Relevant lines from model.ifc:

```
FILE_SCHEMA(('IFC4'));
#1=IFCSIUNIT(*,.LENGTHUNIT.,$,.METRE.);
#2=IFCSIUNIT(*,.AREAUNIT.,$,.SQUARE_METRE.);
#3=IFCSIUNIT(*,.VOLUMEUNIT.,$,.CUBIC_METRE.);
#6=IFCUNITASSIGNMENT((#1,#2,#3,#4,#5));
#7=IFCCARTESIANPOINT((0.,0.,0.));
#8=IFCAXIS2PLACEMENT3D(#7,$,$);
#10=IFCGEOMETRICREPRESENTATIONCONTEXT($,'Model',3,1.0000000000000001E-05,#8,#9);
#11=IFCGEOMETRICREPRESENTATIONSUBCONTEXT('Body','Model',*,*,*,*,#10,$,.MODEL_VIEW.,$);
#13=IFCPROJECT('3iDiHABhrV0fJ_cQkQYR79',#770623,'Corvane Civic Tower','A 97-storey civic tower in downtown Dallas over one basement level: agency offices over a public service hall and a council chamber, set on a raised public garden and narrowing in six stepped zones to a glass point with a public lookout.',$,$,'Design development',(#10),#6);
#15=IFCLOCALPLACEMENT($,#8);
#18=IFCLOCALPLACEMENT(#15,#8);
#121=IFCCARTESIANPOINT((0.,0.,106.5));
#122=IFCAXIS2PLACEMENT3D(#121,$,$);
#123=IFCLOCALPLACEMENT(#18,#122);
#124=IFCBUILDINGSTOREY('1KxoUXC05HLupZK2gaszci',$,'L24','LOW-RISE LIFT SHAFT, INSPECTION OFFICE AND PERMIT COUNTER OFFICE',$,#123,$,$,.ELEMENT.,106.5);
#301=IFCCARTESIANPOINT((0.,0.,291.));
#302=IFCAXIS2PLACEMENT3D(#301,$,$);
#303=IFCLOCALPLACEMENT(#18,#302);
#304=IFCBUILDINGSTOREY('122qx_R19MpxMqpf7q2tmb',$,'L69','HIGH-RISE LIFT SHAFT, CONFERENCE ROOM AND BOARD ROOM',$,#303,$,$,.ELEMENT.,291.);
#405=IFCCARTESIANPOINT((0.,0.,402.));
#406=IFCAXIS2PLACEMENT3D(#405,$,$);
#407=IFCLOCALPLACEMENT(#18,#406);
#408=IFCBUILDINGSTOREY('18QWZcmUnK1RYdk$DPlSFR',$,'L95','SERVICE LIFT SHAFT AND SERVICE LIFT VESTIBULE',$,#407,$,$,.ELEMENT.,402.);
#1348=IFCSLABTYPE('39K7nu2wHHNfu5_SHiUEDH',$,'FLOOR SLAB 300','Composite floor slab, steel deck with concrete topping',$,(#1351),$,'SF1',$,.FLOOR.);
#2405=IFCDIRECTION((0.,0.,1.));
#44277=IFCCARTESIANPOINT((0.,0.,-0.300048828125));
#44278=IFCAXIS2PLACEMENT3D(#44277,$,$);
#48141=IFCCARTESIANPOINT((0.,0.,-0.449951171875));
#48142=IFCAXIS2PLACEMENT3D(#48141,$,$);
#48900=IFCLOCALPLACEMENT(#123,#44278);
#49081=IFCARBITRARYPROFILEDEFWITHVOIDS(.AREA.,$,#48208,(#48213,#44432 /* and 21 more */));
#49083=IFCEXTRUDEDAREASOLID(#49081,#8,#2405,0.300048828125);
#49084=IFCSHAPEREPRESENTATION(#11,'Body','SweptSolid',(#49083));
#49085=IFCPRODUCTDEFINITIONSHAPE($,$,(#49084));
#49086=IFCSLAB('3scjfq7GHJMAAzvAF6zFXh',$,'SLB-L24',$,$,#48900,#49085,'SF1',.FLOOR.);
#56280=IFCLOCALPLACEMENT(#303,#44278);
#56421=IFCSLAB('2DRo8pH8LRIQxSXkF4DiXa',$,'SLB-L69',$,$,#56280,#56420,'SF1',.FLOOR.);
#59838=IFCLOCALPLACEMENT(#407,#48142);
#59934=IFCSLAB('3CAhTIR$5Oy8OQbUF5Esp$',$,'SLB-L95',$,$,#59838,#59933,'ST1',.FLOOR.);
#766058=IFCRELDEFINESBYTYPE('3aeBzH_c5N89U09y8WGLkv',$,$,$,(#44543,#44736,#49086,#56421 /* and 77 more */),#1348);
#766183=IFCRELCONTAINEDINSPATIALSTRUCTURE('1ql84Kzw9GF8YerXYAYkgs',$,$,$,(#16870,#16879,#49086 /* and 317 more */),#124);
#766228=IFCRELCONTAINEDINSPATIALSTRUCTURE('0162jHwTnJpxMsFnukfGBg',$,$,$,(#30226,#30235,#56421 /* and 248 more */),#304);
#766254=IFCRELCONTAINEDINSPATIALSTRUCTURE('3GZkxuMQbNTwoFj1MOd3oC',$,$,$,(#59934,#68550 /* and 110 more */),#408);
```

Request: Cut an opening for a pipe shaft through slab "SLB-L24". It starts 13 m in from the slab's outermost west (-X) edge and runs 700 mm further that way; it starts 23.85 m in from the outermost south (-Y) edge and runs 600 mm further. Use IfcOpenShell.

```python
import numpy as np
import ifcopenshell
import ifcopenshell.api.feature
import ifcopenshell.api.geometry
import ifcopenshell.api.root
import ifcopenshell.geom
import ifcopenshell.util.placement
import ifcopenshell.util.representation
import ifcopenshell.util.shape
import ifcopenshell.util.unit

model = ifcopenshell.open("model.ifc")
unit_scale = ifcopenshell.util.unit.calculate_unit_scale(model)
settings = ifcopenshell.geom.settings()


def volume(element):
    """Net volume in cubic metres, openings subtracted."""
    shape = ifcopenshell.geom.create_shape(settings, element)
    return ifcopenshell.util.shape.get_volume(shape.geometry)


slab = model.by_guid("3scjfq7GHJMAAzvAF6zFXh")
before = volume(slab)

# Extent in the slab's own axes, in metres. The edges named are its -X and -Y sides.
slab_shape = ifcopenshell.geom.create_shape(settings, slab)
vertices = ifcopenshell.util.shape.get_vertices(slab_shape.geometry)
x_min, y_min, bottom = vertices.min(axis=0)
top = vertices[:, 2].max()

opening = ifcopenshell.api.root.create_entity(model, ifc_class="IfcOpeningElement", name="Pipe shaft opening", predefined_type="OPENING")
context = ifcopenshell.util.representation.get_context(model, "Model", "Body", "MODEL_VIEW")
width, depth = 0.7, 0.6
outline = [(0.0, 0.0), (width, 0.0), (width, depth), (0.0, depth), (0.0, 0.0)]
# Overshoot both faces by 50 mm so the cut is clean.
shape = ifcopenshell.api.geometry.add_slab_representation(
    model, context=context, depth=top - bottom + 0.1, polyline=outline
)
ifcopenshell.api.geometry.assign_representation(model, product=opening, representation=shape)

matrix = ifcopenshell.util.placement.get_local_placement(slab.ObjectPlacement)
matrix[:, 3] = matrix @ np.append(np.array([x_min + 13, y_min + 23.85, bottom - 0.05]) / unit_scale, 1.0)
ifcopenshell.api.geometry.edit_object_placement(model, product=opening, matrix=matrix, is_si=False)
ifcopenshell.api.feature.add_feature(model, feature=opening, element=slab)

after = volume(slab)

print(f"slab volume {before:.3f} -> {after:.3f} m3")

model.write("model_updated.ifc")
```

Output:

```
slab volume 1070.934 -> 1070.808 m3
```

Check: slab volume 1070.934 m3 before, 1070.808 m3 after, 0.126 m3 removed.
